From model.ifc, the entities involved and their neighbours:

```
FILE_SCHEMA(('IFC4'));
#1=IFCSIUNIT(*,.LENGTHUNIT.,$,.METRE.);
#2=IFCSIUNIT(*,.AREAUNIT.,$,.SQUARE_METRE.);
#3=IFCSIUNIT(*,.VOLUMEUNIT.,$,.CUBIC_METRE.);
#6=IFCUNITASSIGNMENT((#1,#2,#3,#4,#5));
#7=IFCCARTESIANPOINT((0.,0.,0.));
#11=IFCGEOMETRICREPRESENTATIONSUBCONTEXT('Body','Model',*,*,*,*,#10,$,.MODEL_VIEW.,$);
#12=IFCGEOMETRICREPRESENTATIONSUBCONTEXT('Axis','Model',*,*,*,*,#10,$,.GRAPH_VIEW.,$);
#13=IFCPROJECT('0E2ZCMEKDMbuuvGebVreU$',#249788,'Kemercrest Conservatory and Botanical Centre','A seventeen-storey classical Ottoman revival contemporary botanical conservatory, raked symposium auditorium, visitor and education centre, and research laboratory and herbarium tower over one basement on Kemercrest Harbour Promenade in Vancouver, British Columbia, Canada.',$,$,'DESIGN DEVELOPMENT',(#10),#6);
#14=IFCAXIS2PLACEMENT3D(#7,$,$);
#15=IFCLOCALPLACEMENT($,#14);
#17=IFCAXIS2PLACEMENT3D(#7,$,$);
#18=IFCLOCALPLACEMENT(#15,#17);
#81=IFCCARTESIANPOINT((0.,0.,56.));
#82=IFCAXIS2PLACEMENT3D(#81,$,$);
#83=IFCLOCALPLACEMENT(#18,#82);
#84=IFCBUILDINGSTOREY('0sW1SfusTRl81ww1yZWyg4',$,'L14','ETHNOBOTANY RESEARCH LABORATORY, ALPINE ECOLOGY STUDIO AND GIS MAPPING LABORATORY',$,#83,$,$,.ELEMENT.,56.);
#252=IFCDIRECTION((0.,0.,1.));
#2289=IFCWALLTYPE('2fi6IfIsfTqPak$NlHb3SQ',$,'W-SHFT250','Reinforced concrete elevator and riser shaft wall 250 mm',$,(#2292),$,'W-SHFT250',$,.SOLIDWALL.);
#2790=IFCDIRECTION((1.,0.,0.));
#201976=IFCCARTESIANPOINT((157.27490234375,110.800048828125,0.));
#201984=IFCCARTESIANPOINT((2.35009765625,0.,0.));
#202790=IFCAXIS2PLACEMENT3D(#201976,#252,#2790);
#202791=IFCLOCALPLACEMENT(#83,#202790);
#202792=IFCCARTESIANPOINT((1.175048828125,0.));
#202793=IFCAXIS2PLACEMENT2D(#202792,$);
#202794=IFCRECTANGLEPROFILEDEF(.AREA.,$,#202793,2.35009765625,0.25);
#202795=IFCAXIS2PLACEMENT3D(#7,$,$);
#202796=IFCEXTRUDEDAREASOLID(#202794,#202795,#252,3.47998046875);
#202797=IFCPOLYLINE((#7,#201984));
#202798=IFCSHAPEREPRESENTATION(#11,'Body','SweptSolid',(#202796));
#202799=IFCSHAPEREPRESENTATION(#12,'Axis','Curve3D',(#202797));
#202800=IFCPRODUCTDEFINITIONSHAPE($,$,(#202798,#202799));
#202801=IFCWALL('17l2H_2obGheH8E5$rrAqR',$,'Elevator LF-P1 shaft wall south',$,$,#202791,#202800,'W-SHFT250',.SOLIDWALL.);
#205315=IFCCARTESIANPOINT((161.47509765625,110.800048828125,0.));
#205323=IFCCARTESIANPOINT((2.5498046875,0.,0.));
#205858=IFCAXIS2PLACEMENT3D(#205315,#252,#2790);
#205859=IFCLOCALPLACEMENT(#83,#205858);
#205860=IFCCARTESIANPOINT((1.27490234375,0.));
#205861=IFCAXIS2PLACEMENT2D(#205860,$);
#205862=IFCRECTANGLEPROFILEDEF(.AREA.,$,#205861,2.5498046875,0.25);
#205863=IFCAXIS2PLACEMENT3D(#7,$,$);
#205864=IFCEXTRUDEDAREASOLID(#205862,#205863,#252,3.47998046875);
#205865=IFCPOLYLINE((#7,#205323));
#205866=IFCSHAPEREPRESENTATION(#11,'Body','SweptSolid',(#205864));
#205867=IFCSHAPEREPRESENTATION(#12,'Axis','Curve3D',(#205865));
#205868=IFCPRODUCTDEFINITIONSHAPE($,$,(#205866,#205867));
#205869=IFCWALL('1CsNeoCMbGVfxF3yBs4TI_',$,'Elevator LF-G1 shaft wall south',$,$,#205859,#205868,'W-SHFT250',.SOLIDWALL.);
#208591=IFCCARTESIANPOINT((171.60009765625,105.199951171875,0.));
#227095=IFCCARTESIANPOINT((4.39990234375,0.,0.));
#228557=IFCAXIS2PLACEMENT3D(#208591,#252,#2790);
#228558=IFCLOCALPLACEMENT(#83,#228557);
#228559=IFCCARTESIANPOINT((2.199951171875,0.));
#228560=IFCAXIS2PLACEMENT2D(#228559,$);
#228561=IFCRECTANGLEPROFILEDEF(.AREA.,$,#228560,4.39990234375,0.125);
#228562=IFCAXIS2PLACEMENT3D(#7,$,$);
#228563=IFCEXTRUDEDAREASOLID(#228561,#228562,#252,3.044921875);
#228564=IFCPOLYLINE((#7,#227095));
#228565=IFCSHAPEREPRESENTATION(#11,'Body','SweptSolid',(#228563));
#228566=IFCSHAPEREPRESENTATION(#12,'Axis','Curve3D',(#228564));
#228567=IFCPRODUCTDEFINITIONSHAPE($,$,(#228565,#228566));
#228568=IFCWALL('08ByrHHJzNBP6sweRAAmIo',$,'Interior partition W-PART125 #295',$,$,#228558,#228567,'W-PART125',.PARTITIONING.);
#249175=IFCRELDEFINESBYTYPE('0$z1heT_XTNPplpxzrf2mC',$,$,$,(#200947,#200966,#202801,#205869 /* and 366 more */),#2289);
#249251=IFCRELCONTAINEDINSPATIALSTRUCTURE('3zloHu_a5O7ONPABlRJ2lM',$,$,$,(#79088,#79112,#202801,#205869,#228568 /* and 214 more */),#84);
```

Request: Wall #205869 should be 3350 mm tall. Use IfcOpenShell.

```python
import ifcopenshell
import ifcopenshell.geom
import ifcopenshell.util.representation
import ifcopenshell.util.shape
import ifcopenshell.util.unit

model = ifcopenshell.open("model.ifc")
unit_scale = ifcopenshell.util.unit.calculate_unit_scale(model)
settings = ifcopenshell.geom.settings()


def volume(element):
    """Net volume in cubic metres, openings subtracted."""
    shape = ifcopenshell.geom.create_shape(settings, element)
    return ifcopenshell.util.shape.get_volume(shape.geometry)


wall = model.by_guid("1CsNeoCMbGVfxF3yBs4TI_")
before = volume(wall)

body = ifcopenshell.util.representation.get_representation(wall, "Model", "Body")
solid = body.Items[0]
old_height = solid.Depth
solid.Depth = 3.35 / unit_scale
after = volume(wall)

print(f"height {old_height:g} -> {solid.Depth:g}, volume {before:.3f} -> {after:.3f} m3")

model.write("model_updated.ifc")
```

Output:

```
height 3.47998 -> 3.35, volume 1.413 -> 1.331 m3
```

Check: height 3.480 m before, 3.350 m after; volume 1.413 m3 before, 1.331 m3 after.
